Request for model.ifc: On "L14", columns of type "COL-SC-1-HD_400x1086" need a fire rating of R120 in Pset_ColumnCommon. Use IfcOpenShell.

First a look at what the model holds.

```python
import ifcopenshell
import ifcopenshell.util.element

model = ifcopenshell.open("model.ifc")
print(model.schema)
storey = next(s for s in model.by_type("IfcBuildingStorey") if s.Name == "L14")
columns = [e for e in ifcopenshell.util.element.get_decomposition(storey) if e.is_a("IfcColumn")]
seen = {}
for e in columns:
    element_type = ifcopenshell.util.element.get_type(e)
    key = (element_type.Name if element_type != e and element_type else None, ifcopenshell.util.element.get_pset(e, "Pset_ColumnCommon", "FireRating"))
    seen[key] = seen.get(key, 0) + 1
for (name, value), count in sorted(seen.items(), key=str):
    print(count, "x", name, "|", value)
```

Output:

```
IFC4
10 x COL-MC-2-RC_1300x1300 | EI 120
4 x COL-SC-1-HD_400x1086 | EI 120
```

```python
import ifcopenshell
import ifcopenshell.api.pset
import ifcopenshell.util.element

model = ifcopenshell.open("model.ifc")

storey = next(s for s in model.by_type("IfcBuildingStorey") if s.Name == "L14")
columns = [e for e in ifcopenshell.util.element.get_decomposition(storey) if e.is_a("IfcColumn")]

count = 0
for e in columns:
    element_type = ifcopenshell.util.element.get_type(e)
    if element_type in (None, e) or element_type.Name != "COL-SC-1-HD_400x1086":
        continue
    found = ifcopenshell.util.element.get_pset(e, "Pset_ColumnCommon", should_inherit=False)
    if found:
        pset = model.by_id(found["id"])
        if len(ifcopenshell.util.element.get_elements_by_pset(pset)) > 1:
            pset = ifcopenshell.api.pset.unshare_pset(model, products=[e], pset=pset)[0]
    else:
        pset = ifcopenshell.api.pset.add_pset(model, product=e, name="Pset_ColumnCommon")
    ifcopenshell.api.pset.edit_pset(model, pset=pset, properties={"FireRating": "R120"})
    count += 1

print(count, "columns updated")

model.write("model_updated.ifc")
```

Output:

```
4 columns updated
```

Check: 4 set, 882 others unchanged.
